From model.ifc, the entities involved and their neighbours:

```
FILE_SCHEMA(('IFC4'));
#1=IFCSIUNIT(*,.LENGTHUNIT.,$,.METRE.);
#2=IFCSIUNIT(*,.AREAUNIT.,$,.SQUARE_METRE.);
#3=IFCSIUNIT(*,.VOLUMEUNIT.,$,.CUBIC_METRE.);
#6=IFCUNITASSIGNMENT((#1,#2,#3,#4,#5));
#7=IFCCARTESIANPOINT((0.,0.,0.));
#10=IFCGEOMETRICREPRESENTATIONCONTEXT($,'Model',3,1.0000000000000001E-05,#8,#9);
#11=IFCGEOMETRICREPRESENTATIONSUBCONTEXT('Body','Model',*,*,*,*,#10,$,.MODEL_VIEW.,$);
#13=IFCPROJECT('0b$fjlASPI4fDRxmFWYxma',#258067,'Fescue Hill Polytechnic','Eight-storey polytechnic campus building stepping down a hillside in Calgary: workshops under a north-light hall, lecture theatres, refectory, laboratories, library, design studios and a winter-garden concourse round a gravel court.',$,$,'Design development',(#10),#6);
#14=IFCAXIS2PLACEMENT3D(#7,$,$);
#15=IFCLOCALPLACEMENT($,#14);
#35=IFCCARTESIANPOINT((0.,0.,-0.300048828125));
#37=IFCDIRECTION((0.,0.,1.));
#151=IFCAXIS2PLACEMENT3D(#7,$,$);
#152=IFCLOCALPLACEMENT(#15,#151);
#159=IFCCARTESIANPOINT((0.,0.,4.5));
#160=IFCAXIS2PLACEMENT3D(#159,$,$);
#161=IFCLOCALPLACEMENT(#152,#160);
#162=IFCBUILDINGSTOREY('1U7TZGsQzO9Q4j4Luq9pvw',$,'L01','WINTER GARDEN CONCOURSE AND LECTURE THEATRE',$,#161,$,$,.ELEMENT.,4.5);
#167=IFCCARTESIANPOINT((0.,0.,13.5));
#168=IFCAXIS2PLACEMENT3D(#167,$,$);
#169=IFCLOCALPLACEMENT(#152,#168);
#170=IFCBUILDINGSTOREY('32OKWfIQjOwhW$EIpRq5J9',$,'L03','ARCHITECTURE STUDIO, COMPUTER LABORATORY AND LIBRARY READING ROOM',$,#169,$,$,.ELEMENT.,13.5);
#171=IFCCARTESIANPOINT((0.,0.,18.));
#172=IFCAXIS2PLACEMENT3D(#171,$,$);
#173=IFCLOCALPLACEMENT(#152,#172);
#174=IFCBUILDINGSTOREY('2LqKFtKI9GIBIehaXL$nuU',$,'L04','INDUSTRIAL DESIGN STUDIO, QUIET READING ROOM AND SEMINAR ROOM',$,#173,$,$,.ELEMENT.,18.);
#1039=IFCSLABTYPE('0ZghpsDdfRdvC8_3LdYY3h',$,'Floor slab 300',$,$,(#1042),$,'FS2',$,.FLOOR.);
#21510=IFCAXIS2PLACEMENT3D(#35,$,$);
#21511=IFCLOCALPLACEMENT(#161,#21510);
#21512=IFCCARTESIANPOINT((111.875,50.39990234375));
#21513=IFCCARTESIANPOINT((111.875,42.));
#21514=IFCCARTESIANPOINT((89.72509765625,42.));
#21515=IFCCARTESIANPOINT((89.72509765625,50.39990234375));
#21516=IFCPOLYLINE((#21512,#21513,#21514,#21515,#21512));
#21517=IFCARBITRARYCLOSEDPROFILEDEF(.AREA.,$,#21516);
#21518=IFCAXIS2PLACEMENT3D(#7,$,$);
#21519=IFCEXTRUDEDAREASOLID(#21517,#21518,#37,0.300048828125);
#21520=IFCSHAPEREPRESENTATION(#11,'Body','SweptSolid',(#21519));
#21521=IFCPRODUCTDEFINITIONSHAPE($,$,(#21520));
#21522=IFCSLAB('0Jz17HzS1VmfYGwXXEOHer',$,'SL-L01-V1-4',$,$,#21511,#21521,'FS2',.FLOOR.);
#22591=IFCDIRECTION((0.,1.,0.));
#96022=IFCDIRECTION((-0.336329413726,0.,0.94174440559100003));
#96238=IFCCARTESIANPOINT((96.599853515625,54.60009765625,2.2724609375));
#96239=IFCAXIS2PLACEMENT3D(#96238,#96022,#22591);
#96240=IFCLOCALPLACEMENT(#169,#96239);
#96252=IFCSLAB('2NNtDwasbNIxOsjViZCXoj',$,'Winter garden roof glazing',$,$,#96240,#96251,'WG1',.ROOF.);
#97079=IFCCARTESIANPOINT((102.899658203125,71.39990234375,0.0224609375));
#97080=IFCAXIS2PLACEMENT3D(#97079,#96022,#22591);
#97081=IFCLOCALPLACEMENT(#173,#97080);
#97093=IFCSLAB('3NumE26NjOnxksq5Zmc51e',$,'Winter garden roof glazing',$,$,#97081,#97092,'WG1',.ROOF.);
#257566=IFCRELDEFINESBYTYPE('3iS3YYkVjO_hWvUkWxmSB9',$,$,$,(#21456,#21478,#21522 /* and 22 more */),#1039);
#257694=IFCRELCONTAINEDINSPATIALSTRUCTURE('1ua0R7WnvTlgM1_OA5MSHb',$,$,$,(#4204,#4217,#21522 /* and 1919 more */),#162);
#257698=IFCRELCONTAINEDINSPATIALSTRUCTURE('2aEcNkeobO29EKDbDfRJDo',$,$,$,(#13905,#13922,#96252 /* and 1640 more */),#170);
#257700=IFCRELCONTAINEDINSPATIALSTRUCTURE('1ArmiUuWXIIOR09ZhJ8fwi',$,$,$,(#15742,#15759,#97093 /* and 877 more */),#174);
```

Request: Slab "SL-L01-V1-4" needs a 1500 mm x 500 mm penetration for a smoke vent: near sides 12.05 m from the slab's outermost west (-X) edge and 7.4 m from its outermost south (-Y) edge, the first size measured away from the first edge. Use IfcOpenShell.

```python
import numpy as np
import ifcopenshell
import ifcopenshell.api.feature
import ifcopenshell.api.geometry
import ifcopenshell.api.root
import ifcopenshell.geom
import ifcopenshell.util.placement
import ifcopenshell.util.representation
import ifcopenshell.util.shape
import ifcopenshell.util.unit

model = ifcopenshell.open("model.ifc")
unit_scale = ifcopenshell.util.unit.calculate_unit_scale(model)
settings = ifcopenshell.geom.settings()


def volume(element):
    """Net volume in cubic metres, openings subtracted."""
    shape = ifcopenshell.geom.create_shape(settings, element)
    return ifcopenshell.util.shape.get_volume(shape.geometry)


slab = model.by_guid("0Jz17HzS1VmfYGwXXEOHer")
before = volume(slab)

# Extent in the slab's own axes, in metres. The edges named are its -X and -Y sides.
slab_shape = ifcopenshell.geom.create_shape(settings, slab)
vertices = ifcopenshell.util.shape.get_vertices(slab_shape.geometry)
x_min, y_min, bottom = vertices.min(axis=0)
top = vertices[:, 2].max()

opening = ifcopenshell.api.root.create_entity(model, ifc_class="IfcOpeningElement", name="Smoke vent opening", predefined_type="OPENING")
context = ifcopenshell.util.representation.get_context(model, "Model", "Body", "MODEL_VIEW")
width, depth = 1.5, 0.5
outline = [(0.0, 0.0), (width, 0.0), (width, depth), (0.0, depth), (0.0, 0.0)]
# Overshoot both faces by 50 mm so the cut is clean.
shape = ifcopenshell.api.geometry.add_slab_representation(
    model, context=context, depth=top - bottom + 0.1, polyline=outline
)
ifcopenshell.api.geometry.assign_representation(model, product=opening, representation=shape)

matrix = ifcopenshell.util.placement.get_local_placement(slab.ObjectPlacement)
matrix[:, 3] = matrix @ np.append(np.array([x_min + 12.05, y_min + 7.4, bottom - 0.05]) / unit_scale, 1.0)
ifcopenshell.api.geometry.edit_object_placement(model, product=opening, matrix=matrix, is_si=False)
ifcopenshell.api.feature.add_feature(model, feature=opening, element=slab)

after = volume(slab)

print(f"slab volume {before:.3f} -> {after:.3f} m3")

model.write("model_rev.ifc")
```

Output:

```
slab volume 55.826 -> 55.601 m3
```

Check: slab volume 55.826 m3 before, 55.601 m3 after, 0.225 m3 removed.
